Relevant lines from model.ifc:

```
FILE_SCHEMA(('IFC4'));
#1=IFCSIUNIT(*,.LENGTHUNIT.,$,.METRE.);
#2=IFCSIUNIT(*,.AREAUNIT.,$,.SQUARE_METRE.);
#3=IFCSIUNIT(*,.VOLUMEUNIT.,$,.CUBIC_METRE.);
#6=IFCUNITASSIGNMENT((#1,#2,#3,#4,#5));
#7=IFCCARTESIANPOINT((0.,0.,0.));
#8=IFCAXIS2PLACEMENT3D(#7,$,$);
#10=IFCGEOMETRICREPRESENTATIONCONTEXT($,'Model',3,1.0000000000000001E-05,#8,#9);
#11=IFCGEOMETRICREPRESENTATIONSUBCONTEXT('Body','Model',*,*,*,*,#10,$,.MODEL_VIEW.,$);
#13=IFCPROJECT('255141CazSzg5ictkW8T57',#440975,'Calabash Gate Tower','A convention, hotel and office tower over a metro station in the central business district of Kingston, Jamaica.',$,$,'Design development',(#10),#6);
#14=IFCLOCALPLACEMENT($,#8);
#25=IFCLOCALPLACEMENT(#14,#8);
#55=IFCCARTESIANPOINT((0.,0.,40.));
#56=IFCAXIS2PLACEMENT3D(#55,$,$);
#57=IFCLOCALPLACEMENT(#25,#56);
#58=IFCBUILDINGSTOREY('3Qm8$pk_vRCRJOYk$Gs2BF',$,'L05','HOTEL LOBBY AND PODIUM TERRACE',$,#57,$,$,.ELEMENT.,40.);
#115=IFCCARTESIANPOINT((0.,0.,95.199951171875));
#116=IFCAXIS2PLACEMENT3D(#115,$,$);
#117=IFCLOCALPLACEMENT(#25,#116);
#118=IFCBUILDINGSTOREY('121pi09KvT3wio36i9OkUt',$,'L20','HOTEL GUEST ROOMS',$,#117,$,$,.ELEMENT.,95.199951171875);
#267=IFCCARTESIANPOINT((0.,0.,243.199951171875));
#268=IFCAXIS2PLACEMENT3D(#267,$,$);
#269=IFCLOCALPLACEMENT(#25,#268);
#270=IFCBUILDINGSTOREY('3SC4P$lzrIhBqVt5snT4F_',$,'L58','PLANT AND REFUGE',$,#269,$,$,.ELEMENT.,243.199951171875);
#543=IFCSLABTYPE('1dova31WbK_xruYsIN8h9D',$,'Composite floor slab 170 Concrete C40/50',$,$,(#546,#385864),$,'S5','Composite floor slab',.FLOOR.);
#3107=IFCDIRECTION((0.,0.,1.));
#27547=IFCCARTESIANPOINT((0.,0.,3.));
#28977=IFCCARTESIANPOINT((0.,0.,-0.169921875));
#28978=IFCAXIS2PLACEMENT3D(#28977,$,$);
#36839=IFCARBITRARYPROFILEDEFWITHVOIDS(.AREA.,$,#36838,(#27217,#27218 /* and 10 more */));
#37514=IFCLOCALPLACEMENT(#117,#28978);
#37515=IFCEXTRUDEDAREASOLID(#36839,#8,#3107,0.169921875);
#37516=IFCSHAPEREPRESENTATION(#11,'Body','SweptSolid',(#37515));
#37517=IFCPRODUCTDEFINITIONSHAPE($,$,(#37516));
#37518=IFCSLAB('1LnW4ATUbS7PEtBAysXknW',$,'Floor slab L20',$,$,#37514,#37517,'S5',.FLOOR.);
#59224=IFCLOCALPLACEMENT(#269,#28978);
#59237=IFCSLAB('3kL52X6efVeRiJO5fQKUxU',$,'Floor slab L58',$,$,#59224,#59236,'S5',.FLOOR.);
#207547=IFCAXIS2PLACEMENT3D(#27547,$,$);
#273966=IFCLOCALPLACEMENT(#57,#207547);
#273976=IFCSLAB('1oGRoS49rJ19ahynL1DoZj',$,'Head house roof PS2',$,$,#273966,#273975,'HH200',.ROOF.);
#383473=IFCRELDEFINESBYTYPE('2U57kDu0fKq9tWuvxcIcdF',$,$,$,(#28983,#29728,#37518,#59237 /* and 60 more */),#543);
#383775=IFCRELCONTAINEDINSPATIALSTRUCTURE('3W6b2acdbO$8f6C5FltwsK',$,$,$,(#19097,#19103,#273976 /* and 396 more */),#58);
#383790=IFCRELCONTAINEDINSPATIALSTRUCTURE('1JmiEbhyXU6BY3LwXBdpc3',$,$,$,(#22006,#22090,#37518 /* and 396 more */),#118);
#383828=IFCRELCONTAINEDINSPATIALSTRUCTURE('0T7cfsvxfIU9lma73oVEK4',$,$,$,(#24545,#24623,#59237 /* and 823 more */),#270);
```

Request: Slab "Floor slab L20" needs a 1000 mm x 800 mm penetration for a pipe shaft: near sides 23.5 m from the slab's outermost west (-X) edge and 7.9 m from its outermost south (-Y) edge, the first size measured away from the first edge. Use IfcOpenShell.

```python
import numpy as np
import ifcopenshell
import ifcopenshell.api.feature
import ifcopenshell.api.geometry
import ifcopenshell.api.root
import ifcopenshell.geom
import ifcopenshell.util.placement
import ifcopenshell.util.representation
import ifcopenshell.util.shape
import ifcopenshell.util.unit

model = ifcopenshell.open("model.ifc")
unit_scale = ifcopenshell.util.unit.calculate_unit_scale(model)
settings = ifcopenshell.geom.settings()


def volume(element):
    """Net volume in cubic metres, openings subtracted."""
    shape = ifcopenshell.geom.create_shape(settings, element)
    return ifcopenshell.util.shape.get_volume(shape.geometry)


slab = model.by_guid("1LnW4ATUbS7PEtBAysXknW")
before = volume(slab)

# Extent in the slab's own axes, in metres. The edges named are its -X and -Y sides.
slab_shape = ifcopenshell.geom.create_shape(settings, slab)
vertices = ifcopenshell.util.shape.get_vertices(slab_shape.geometry)
x_min, y_min, bottom = vertices.min(axis=0)
top = vertices[:, 2].max()

opening = ifcopenshell.api.root.create_entity(model, ifc_class="IfcOpeningElement", name="Pipe shaft opening", predefined_type="OPENING")
context = ifcopenshell.util.representation.get_context(model, "Model", "Body", "MODEL_VIEW")
width, depth = 1, 0.8
outline = [(0.0, 0.0), (width, 0.0), (width, depth), (0.0, depth), (0.0, 0.0)]
# Overshoot both faces by 50 mm so the cut is clean.
shape = ifcopenshell.api.geometry.add_slab_representation(
    model, context=context, depth=top - bottom + 0.1, polyline=outline
)
ifcopenshell.api.geometry.assign_representation(model, product=opening, representation=shape)

matrix = ifcopenshell.util.placement.get_local_placement(slab.ObjectPlacement)
matrix[:, 3] = matrix @ np.append(np.array([x_min + 23.5, y_min + 7.9, bottom - 0.05]) / unit_scale, 1.0)
ifcopenshell.api.geometry.edit_object_placement(model, product=opening, matrix=matrix, is_si=False)
ifcopenshell.api.feature.add_feature(model, feature=opening, element=slab)

after = volume(slab)

print(f"slab volume {before:.3f} -> {after:.3f} m3")

model.write("model_updated.ifc")
```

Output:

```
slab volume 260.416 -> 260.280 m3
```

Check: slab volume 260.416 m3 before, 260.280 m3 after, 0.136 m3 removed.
